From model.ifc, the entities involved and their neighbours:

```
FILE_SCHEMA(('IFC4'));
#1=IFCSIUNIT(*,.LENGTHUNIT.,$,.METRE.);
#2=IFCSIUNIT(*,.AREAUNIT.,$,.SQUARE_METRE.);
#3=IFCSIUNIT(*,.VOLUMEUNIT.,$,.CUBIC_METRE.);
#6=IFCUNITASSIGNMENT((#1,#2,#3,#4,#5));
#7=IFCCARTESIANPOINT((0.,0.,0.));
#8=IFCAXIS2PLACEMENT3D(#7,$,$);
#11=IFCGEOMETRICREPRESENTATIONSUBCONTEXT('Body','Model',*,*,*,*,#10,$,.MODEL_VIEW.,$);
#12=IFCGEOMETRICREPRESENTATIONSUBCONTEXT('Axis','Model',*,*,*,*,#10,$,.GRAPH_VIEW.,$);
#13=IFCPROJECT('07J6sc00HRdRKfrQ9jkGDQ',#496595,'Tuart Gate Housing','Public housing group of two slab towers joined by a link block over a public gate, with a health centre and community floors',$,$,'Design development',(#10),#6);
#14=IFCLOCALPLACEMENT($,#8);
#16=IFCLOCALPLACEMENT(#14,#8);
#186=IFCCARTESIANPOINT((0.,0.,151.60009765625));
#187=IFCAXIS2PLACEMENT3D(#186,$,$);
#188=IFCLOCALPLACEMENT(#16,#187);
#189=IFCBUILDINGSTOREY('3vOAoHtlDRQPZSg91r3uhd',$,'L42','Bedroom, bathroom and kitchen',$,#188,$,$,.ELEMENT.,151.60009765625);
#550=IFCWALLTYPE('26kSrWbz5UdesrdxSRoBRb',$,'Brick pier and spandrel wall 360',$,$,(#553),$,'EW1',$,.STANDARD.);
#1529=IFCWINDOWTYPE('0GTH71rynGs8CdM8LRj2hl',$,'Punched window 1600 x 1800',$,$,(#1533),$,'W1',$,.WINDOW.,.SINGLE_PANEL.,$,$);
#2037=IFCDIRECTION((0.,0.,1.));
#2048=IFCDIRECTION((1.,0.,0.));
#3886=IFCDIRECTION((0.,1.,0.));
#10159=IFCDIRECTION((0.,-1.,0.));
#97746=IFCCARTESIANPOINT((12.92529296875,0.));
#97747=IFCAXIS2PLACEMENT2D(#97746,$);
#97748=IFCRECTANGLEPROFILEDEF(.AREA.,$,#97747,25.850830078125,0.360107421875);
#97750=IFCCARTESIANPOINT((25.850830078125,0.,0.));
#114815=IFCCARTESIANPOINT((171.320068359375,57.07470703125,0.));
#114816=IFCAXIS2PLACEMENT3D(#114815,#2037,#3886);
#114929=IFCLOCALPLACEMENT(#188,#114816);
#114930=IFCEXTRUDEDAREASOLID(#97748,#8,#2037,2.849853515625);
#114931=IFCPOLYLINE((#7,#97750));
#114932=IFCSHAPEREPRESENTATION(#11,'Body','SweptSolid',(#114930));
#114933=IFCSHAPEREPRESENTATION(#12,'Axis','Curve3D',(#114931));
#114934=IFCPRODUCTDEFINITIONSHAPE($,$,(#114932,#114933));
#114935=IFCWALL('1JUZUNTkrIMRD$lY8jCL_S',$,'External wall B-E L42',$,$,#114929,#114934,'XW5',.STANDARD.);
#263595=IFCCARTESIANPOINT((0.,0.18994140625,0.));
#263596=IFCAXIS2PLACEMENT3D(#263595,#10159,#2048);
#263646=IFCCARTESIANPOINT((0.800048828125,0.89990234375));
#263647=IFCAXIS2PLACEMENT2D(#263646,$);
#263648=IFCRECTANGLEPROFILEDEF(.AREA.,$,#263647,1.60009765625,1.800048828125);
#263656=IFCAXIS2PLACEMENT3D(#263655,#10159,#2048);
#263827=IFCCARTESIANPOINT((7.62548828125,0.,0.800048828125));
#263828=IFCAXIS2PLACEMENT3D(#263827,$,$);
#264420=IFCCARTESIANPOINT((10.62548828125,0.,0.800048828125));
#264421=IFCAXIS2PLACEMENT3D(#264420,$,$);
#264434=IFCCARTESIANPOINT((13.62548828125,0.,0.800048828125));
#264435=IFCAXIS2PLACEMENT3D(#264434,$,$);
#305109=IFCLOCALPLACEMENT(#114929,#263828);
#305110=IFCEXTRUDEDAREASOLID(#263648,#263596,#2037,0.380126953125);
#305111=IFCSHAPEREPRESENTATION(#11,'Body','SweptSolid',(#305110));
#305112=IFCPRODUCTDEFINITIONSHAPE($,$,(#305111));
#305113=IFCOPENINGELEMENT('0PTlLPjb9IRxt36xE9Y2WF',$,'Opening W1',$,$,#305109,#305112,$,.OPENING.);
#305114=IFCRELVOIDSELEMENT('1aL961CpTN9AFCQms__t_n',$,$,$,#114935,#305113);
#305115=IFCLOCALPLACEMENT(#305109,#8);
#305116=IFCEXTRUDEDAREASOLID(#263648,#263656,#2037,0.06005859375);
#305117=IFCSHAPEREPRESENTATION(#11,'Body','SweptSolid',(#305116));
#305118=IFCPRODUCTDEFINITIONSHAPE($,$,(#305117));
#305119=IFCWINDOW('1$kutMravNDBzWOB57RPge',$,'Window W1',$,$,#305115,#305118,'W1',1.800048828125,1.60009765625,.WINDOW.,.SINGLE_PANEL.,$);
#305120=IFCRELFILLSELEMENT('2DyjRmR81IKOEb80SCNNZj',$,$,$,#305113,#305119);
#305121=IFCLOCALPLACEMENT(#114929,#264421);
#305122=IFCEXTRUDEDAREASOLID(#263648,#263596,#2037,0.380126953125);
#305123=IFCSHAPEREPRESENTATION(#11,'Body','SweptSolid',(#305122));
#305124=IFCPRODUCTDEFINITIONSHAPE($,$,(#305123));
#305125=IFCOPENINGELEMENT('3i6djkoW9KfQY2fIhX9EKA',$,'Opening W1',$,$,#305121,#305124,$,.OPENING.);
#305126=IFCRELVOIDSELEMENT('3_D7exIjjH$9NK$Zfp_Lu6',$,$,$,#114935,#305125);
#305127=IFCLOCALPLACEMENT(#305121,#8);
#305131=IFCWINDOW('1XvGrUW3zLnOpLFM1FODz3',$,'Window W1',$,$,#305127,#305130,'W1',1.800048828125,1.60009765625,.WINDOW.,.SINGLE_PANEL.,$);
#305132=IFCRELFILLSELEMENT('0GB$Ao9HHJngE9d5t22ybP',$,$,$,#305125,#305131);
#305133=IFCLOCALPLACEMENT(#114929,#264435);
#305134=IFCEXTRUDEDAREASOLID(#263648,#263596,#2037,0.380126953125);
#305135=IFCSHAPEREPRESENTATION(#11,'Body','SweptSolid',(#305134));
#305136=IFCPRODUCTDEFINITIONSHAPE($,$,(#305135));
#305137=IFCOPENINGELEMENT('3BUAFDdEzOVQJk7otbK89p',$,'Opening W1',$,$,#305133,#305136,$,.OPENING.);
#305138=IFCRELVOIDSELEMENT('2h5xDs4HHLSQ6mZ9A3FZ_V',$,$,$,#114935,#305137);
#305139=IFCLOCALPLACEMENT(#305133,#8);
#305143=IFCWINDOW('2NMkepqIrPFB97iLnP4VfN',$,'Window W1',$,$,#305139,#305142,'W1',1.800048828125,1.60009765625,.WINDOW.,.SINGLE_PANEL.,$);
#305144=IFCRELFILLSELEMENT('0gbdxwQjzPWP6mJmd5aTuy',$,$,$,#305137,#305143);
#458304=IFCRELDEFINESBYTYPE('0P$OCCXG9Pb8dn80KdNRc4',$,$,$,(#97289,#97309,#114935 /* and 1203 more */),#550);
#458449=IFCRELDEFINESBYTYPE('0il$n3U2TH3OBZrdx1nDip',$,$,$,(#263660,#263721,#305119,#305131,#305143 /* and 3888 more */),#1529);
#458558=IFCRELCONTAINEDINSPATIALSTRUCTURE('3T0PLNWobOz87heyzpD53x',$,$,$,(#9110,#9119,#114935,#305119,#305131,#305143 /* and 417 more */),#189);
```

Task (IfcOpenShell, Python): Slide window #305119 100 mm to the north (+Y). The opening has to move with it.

```python
import ifcopenshell
import ifcopenshell.api.geometry
import ifcopenshell.util.placement

model = ifcopenshell.open("model.ifc")

window = model.by_guid("1$kutMravNDBzWOB57RPge")
opening = window.FillsVoids[0].RelatingOpeningElement
wall = opening.VoidsElements[0].RelatingBuildingElement

wall_matrix = ifcopenshell.util.placement.get_local_placement(wall.ObjectPlacement)
shift = wall_matrix[:3, 0] * 0.1
before = ifcopenshell.util.placement.get_local_placement(window.ObjectPlacement)[:3, 3].copy()

# The window is placed relative to its opening, so it follows when the opening moves.
matrix = ifcopenshell.util.placement.get_local_placement(opening.ObjectPlacement)
matrix[:3, 3] += shift
ifcopenshell.api.geometry.edit_object_placement(
    model, product=opening, matrix=matrix, is_si=False, should_transform_children=True
)

after = ifcopenshell.util.placement.get_local_placement(window.ObjectPlacement)[:3, 3]
print("window moved by", (after - before).round(3) + 0.0)

model.write("model-out.ifc")
```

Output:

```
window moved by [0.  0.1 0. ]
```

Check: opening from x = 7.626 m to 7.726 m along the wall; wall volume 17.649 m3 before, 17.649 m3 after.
